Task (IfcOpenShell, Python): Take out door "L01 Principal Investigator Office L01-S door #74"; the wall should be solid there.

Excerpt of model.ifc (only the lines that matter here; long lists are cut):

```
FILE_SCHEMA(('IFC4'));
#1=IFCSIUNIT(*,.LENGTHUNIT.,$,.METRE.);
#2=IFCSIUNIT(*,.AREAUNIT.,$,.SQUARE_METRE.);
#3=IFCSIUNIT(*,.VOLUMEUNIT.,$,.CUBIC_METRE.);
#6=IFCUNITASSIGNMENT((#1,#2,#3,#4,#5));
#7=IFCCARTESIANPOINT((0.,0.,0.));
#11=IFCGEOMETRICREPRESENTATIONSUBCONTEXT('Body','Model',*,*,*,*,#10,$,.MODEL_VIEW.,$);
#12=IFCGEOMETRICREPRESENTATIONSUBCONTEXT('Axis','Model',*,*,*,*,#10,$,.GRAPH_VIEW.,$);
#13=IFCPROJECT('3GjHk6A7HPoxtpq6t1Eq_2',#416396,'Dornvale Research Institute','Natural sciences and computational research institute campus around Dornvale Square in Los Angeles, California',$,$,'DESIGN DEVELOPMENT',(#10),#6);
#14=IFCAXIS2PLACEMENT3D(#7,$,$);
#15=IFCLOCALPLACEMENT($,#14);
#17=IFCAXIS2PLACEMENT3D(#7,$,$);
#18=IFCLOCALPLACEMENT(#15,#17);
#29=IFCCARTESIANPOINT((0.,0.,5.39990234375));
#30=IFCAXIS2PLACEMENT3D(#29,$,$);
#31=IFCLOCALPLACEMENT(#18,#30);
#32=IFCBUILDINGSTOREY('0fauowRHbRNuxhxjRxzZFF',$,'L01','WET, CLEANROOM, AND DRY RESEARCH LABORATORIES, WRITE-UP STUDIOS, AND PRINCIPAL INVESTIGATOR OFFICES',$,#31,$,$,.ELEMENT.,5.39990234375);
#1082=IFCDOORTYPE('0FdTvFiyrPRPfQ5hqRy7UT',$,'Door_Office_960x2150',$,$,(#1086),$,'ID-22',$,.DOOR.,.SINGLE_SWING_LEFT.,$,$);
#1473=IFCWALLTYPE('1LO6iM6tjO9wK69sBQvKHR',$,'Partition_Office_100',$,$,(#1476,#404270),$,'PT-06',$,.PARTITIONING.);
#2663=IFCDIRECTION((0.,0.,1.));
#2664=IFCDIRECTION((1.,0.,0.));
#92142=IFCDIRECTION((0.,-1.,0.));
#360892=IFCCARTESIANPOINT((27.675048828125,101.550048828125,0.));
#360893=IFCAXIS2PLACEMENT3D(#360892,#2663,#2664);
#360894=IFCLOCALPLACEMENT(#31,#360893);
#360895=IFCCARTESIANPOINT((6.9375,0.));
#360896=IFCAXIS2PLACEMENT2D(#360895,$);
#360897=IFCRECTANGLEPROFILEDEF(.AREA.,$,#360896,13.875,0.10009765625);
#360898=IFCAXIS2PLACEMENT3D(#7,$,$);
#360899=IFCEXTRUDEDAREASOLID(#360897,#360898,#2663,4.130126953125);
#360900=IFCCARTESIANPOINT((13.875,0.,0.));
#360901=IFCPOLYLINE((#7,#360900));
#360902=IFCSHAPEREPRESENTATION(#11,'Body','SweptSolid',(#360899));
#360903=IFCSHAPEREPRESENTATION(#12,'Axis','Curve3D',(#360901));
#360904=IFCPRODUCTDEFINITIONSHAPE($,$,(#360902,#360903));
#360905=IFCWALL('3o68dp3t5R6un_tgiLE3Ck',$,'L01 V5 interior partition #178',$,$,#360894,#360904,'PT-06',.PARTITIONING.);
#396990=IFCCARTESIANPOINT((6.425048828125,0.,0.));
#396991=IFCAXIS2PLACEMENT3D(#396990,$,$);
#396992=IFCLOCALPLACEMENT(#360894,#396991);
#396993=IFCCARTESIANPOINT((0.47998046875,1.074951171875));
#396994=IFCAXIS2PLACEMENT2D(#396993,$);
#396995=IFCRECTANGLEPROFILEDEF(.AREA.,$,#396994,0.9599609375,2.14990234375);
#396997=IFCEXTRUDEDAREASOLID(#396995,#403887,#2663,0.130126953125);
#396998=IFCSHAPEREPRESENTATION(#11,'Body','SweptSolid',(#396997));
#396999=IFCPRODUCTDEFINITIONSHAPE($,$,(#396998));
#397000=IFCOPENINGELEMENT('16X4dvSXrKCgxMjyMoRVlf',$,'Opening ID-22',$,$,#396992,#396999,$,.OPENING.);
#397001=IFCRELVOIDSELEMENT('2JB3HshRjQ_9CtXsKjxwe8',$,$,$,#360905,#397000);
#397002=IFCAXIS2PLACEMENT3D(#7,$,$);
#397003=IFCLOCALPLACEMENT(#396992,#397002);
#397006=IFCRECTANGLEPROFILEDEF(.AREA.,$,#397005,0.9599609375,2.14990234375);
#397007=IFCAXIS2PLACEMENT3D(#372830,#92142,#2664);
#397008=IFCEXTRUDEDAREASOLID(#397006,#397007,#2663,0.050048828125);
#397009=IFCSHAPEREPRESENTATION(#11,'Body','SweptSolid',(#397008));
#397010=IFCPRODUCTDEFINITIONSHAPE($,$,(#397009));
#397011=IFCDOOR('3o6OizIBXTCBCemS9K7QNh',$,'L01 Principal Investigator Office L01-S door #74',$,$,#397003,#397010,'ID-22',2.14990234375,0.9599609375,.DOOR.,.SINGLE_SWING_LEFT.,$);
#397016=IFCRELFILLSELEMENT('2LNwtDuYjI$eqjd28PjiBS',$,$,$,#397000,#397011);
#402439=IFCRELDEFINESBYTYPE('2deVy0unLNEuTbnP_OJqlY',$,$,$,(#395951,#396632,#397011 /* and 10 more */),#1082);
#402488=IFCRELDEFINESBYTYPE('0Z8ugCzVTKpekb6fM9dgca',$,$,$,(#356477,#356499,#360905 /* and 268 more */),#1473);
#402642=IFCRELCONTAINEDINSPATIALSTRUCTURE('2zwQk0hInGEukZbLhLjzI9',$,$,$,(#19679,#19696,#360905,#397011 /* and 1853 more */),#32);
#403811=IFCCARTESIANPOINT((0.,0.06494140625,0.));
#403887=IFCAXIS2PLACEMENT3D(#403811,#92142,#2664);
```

```python
import ifcopenshell
import ifcopenshell.api.feature
import ifcopenshell.api.root
import ifcopenshell.geom
import ifcopenshell.util.shape

model = ifcopenshell.open("model.ifc")
settings = ifcopenshell.geom.settings()


def volume(element):
    """Net volume in cubic metres, openings subtracted."""
    shape = ifcopenshell.geom.create_shape(settings, element)
    return ifcopenshell.util.shape.get_volume(shape.geometry)


door = model.by_guid("3o6OizIBXTCBCemS9K7QNh")
opening = door.FillsVoids[0].RelatingOpeningElement
wall = opening.VoidsElements[0].RelatingBuildingElement
before = volume(wall)

ifcopenshell.api.root.remove_product(model, product=door)
ifcopenshell.api.feature.remove_feature(model, feature=opening)

after = volume(wall)

print(f"wall volume {before:.3f} -> {after:.3f} m3")

model.write("model_edited.ifc")
```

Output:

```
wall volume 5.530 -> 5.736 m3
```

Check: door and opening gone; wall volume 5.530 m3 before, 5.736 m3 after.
